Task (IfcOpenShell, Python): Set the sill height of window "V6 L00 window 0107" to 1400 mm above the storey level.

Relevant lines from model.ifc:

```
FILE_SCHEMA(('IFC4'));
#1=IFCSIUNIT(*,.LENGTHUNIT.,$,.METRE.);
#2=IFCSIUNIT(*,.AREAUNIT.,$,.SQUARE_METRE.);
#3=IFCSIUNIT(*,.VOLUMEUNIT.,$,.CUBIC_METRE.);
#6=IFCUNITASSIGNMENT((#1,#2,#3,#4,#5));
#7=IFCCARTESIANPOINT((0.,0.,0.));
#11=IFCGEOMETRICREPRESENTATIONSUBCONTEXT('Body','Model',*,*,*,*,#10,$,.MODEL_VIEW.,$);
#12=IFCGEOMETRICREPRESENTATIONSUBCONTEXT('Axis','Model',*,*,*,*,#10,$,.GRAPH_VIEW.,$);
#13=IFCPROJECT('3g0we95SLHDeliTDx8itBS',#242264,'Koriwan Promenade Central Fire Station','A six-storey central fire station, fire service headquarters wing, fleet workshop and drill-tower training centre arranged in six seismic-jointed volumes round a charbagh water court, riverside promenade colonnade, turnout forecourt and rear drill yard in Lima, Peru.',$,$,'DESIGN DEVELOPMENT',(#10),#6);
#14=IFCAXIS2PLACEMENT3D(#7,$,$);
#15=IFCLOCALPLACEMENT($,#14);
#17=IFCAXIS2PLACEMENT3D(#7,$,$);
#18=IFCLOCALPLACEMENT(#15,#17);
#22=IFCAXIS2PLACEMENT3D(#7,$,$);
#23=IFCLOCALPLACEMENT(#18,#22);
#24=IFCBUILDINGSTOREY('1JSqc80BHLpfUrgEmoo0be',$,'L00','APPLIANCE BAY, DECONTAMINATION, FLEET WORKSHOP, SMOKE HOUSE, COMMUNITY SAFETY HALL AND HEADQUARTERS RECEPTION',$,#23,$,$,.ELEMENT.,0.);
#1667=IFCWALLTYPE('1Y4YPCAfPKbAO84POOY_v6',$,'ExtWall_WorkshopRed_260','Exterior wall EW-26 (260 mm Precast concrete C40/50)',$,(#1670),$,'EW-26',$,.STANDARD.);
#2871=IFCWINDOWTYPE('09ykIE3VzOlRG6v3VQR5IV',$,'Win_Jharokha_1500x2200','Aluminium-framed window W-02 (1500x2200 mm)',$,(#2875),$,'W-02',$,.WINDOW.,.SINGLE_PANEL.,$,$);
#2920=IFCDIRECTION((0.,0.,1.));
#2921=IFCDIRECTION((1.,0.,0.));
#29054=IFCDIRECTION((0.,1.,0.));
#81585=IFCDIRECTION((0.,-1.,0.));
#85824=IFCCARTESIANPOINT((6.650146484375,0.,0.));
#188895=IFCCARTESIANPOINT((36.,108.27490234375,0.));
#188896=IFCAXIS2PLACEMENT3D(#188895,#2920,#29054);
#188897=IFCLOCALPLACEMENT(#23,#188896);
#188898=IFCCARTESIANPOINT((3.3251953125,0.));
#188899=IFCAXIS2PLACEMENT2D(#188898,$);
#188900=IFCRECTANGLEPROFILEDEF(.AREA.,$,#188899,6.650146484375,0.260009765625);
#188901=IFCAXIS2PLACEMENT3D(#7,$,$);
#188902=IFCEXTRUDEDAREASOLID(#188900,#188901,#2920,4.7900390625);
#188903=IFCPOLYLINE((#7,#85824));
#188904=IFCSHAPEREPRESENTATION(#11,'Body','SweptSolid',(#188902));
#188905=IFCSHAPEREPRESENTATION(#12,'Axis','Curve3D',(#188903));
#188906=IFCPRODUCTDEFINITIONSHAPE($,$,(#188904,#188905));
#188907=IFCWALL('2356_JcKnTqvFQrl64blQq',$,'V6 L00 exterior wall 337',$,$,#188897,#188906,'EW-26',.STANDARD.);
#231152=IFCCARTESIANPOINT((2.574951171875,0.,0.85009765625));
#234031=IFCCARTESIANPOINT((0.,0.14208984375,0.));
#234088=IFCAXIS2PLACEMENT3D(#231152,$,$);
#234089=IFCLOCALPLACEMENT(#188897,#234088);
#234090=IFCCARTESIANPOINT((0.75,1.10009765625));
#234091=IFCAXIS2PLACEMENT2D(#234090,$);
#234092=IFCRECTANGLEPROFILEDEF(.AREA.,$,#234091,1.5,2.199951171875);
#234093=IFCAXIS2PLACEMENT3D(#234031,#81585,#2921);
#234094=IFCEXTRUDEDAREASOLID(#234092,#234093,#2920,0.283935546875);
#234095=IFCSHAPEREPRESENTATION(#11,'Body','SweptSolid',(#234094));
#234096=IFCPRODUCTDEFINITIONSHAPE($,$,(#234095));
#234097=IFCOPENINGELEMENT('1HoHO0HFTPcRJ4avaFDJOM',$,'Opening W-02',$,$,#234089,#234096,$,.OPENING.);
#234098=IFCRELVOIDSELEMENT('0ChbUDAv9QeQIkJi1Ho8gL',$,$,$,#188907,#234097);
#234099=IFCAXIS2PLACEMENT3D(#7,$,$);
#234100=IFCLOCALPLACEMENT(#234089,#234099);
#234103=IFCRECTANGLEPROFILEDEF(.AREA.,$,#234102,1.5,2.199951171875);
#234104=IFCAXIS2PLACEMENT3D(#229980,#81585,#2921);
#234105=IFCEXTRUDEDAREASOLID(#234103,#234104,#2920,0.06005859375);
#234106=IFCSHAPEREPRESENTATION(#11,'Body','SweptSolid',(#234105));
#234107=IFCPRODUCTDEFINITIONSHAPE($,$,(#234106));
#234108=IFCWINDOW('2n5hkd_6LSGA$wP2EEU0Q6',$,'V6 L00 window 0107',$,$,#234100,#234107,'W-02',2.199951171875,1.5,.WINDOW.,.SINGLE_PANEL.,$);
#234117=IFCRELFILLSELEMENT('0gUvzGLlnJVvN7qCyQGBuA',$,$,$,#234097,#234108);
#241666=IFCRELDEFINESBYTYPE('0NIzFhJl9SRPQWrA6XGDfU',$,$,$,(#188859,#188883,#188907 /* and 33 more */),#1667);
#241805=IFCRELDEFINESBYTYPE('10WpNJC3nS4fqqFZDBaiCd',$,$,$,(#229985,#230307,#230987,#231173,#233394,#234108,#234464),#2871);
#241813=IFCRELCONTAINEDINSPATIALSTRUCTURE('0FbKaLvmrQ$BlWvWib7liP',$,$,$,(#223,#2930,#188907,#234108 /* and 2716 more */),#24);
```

```python
import numpy as np
import ifcopenshell
import ifcopenshell.api.geometry
import ifcopenshell.geom
import ifcopenshell.util.element
import ifcopenshell.util.placement
import ifcopenshell.util.shape
import ifcopenshell.util.unit

model = ifcopenshell.open("model.ifc")
unit_scale = ifcopenshell.util.unit.calculate_unit_scale(model)

window = model.by_guid("2n5hkd_6LSGA$wP2EEU0Q6")
opening = window.FillsVoids[0].RelatingOpeningElement
storey = ifcopenshell.util.element.get_container(window, ifc_class="IfcBuildingStorey")
level = ifcopenshell.util.placement.get_local_placement(storey.ObjectPlacement)[2, 3]

# The opening's origin need not be at the sill, so measure its lowest point.
shape = ifcopenshell.geom.create_shape(ifcopenshell.geom.settings(), opening)
bottom = ifcopenshell.util.shape.get_shape_bottom_elevation(shape, shape.geometry) / unit_scale
dz = level + 1.4 - bottom

shift = np.array([0.0, 0.0, dz])
# The window is placed relative to its opening, so it follows when the opening moves.
matrix = ifcopenshell.util.placement.get_local_placement(opening.ObjectPlacement)
matrix[:3, 3] += shift
ifcopenshell.api.geometry.edit_object_placement(
    model, product=opening, matrix=matrix, is_si=False, should_transform_children=True
)

print(f"moved by {dz * unit_scale:+.3f} m")

model.write("model_updated.ifc")
```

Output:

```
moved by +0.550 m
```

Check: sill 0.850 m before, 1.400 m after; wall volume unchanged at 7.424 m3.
